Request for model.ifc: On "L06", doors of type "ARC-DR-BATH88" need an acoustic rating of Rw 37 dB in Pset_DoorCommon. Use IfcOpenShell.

First a look at what the model holds.

```python
import ifcopenshell
import ifcopenshell.util.element

model = ifcopenshell.open("model.ifc")
print(model.schema)
storey = next(s for s in model.by_type("IfcBuildingStorey") if s.Name == "L06")
doors = [e for e in ifcopenshell.util.element.get_decomposition(storey) if e.is_a("IfcDoor")]
seen = {}
for e in doors:
    element_type = ifcopenshell.util.element.get_type(e)
    key = (element_type.Name if element_type != e and element_type else None, ifcopenshell.util.element.get_pset(e, "Pset_DoorCommon", "AcousticRating"))
    seen[key] = seen.get(key, 0) + 1
for (name, value), count in sorted(seen.items(), key=str):
    print(count, "x", name, "|", value)
```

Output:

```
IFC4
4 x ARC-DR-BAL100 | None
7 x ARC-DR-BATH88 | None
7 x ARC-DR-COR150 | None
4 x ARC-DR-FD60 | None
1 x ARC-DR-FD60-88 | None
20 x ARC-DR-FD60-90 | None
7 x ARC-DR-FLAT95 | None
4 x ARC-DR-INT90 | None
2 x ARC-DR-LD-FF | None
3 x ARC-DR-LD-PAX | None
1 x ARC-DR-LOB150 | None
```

```python
import ifcopenshell
import ifcopenshell.api.pset
import ifcopenshell.util.element

model = ifcopenshell.open("model.ifc")

storey = next(s for s in model.by_type("IfcBuildingStorey") if s.Name == "L06")
doors = [e for e in ifcopenshell.util.element.get_decomposition(storey) if e.is_a("IfcDoor")]

count = 0
for e in doors:
    element_type = ifcopenshell.util.element.get_type(e)
    if element_type in (None, e) or element_type.Name != "ARC-DR-BATH88":
        continue
    found = ifcopenshell.util.element.get_pset(e, "Pset_DoorCommon", should_inherit=False)
    if found:
        pset = model.by_id(found["id"])
        if len(ifcopenshell.util.element.get_elements_by_pset(pset)) > 1:
            pset = ifcopenshell.api.pset.unshare_pset(model, products=[e], pset=pset)[0]
    else:
        pset = ifcopenshell.api.pset.add_pset(model, product=e, name="Pset_DoorCommon")
    ifcopenshell.api.pset.edit_pset(model, pset=pset, properties={"AcousticRating": "Rw 37 dB"})
    count += 1

print(count, "doors updated")

model.write("model_v2.ifc")
```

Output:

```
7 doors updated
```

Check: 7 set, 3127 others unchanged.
